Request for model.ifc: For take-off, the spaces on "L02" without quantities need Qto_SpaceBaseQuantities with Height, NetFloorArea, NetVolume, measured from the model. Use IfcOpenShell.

First a look at what the model holds.

```python
import ifcopenshell
import ifcopenshell.util.element
import ifcopenshell.util.unit

model = ifcopenshell.open("model.ifc")
print(model.schema)
for unit_type in ("LENGTHUNIT", "AREAUNIT", "VOLUMEUNIT"):
    print(unit_type, ifcopenshell.util.unit.calculate_unit_scale(model, unit_type))
storey = next(s for s in model.by_type("IfcBuildingStorey") if s.Name == "L02")
spaces = [e for e in ifcopenshell.util.element.get_decomposition(storey) if e.is_a("IfcSpace")]
for e in sorted(spaces, key=lambda e: e.id()):
    print(e.id(), e.is_a(), e.Name, list(ifcopenshell.util.element.get_psets(e, qtos_only=True)), sep=" | ")
```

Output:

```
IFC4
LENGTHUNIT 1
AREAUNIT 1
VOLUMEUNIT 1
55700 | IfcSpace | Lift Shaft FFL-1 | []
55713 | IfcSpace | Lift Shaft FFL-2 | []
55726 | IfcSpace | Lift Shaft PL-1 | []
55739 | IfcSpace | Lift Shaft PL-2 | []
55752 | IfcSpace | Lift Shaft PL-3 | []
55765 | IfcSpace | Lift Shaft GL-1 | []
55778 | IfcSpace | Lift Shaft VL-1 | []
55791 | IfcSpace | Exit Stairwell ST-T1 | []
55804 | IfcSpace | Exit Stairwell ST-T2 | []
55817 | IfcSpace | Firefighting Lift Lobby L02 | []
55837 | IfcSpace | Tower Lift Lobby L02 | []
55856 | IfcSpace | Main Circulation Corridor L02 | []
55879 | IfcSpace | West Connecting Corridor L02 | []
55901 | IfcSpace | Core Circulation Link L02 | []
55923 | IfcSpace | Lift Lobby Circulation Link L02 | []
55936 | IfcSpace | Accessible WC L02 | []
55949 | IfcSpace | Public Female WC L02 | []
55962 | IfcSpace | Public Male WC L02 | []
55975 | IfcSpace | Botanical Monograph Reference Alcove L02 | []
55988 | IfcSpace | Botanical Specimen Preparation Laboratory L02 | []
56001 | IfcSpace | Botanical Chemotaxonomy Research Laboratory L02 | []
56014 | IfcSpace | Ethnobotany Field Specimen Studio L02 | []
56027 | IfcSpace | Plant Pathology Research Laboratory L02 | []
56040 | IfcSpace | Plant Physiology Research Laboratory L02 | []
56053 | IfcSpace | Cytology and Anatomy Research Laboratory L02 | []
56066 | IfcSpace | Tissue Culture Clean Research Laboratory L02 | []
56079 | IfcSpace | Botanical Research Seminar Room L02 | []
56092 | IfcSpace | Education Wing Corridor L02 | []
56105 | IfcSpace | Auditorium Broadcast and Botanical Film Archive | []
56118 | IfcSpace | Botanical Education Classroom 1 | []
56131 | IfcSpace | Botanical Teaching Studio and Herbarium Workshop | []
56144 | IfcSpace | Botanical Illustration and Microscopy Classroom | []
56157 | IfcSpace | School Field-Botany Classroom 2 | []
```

```python
import ifcopenshell
import ifcopenshell.api.pset
import ifcopenshell.geom
import ifcopenshell.util.element
import ifcopenshell.util.shape
import ifcopenshell.util.unit

model = ifcopenshell.open("model.ifc")
unit_scale = ifcopenshell.util.unit.calculate_unit_scale(model)
area_scale = ifcopenshell.util.unit.calculate_unit_scale(model, "AREAUNIT")
volume_scale = ifcopenshell.util.unit.calculate_unit_scale(model, "VOLUMEUNIT")
settings = ifcopenshell.geom.settings()

storey = next(s for s in model.by_type("IfcBuildingStorey") if s.Name == "L02")
spaces = [e for e in ifcopenshell.util.element.get_decomposition(storey) if e.is_a("IfcSpace")]

for e in sorted(spaces, key=lambda e: e.id()):
    if ifcopenshell.util.element.get_psets(e, qtos_only=True, should_inherit=False):
        continue
    # Geometry comes back in metres, in the element's own axes.
    shape = ifcopenshell.geom.create_shape(settings, e)
    values = {
        "Height": ifcopenshell.util.shape.get_z(shape.geometry) / unit_scale,
        "NetFloorArea": ifcopenshell.util.shape.get_footprint_area(shape.geometry) / area_scale,
        "NetVolume": ifcopenshell.util.shape.get_volume(shape.geometry) / volume_scale,
    }
    qto = ifcopenshell.api.pset.add_qto(model, product=e, name="Qto_SpaceBaseQuantities")
    ifcopenshell.api.pset.edit_qto(model, qto=qto, properties=values)
    print(e.id(), {k: round(v, 3) for k, v in values.items()})

model.write("model_rev.ifc")
```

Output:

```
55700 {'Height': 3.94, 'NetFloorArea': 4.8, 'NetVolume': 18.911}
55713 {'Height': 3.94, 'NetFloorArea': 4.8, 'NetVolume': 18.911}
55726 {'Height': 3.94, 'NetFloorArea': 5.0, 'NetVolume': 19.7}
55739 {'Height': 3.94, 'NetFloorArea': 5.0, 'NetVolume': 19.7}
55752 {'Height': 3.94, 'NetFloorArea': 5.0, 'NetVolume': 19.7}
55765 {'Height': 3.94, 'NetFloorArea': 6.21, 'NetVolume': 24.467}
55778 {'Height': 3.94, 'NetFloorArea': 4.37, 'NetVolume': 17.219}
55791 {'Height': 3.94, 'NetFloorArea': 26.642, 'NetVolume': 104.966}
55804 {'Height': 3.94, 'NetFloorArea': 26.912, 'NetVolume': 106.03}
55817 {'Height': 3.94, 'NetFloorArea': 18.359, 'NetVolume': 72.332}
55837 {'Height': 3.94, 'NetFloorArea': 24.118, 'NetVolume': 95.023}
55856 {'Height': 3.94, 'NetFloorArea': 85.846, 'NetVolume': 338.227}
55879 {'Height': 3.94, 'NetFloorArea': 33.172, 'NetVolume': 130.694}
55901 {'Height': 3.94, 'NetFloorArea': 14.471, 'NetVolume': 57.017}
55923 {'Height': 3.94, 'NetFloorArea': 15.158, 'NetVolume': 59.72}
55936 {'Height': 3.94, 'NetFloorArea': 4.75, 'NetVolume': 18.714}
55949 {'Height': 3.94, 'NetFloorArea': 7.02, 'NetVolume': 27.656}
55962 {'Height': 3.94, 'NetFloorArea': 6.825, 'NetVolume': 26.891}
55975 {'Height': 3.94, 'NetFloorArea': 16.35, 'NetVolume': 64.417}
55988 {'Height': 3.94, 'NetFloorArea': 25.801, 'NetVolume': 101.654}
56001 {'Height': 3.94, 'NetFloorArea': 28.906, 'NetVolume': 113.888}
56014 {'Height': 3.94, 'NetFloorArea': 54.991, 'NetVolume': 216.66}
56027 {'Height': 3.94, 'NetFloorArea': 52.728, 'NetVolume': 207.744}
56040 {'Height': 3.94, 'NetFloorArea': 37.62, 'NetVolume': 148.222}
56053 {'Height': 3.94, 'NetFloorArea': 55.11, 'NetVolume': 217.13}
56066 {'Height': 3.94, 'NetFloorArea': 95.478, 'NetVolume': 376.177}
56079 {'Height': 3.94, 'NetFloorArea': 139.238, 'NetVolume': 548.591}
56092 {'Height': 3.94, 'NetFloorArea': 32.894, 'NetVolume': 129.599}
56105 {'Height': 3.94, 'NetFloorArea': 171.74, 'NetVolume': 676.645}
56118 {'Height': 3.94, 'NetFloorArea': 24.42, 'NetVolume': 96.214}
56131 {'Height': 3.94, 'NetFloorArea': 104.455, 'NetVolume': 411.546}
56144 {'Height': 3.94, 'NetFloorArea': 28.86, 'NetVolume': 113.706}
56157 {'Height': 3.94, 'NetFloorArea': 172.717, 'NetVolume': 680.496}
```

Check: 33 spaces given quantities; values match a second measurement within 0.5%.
